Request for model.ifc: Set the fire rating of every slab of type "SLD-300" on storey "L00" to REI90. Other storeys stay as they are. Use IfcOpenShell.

First a look at what the model holds.

```python
import ifcopenshell
import ifcopenshell.util.element

model = ifcopenshell.open("model.ifc")
print(model.schema)
storey = next(s for s in model.by_type("IfcBuildingStorey") if s.Name == "L00")
slabs = [e for e in ifcopenshell.util.element.get_decomposition(storey) if e.is_a("IfcSlab")]
seen = {}
for e in slabs:
    element_type = ifcopenshell.util.element.get_type(e)
    key = (element_type.Name if element_type != e and element_type else None, ifcopenshell.util.element.get_pset(e, "Pset_SlabCommon", "FireRating"))
    seen[key] = seen.get(key, 0) + 1
for (name, value), count in sorted(seen.items(), key=str):
    print(count, "x", name, "|", value)
```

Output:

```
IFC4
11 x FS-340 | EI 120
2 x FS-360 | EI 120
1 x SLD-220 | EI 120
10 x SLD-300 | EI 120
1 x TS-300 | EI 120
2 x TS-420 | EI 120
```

```python
import ifcopenshell
import ifcopenshell.api.pset
import ifcopenshell.util.element

model = ifcopenshell.open("model.ifc")

storey = next(s for s in model.by_type("IfcBuildingStorey") if s.Name == "L00")
slabs = [e for e in ifcopenshell.util.element.get_decomposition(storey) if e.is_a("IfcSlab")]

count = 0
for e in slabs:
    element_type = ifcopenshell.util.element.get_type(e)
    if element_type in (None, e) or element_type.Name != "SLD-300":
        continue
    # add_pset returns the element's existing set when there is one.
    pset = ifcopenshell.api.pset.add_pset(model, product=e, name="Pset_SlabCommon")
    ifcopenshell.api.pset.edit_pset(model, pset=pset, properties={"FireRating": "REI90"})
    count += 1

print(count, "slabs updated")

model.write("model_rev.ifc")
```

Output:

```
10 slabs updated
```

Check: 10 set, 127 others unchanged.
